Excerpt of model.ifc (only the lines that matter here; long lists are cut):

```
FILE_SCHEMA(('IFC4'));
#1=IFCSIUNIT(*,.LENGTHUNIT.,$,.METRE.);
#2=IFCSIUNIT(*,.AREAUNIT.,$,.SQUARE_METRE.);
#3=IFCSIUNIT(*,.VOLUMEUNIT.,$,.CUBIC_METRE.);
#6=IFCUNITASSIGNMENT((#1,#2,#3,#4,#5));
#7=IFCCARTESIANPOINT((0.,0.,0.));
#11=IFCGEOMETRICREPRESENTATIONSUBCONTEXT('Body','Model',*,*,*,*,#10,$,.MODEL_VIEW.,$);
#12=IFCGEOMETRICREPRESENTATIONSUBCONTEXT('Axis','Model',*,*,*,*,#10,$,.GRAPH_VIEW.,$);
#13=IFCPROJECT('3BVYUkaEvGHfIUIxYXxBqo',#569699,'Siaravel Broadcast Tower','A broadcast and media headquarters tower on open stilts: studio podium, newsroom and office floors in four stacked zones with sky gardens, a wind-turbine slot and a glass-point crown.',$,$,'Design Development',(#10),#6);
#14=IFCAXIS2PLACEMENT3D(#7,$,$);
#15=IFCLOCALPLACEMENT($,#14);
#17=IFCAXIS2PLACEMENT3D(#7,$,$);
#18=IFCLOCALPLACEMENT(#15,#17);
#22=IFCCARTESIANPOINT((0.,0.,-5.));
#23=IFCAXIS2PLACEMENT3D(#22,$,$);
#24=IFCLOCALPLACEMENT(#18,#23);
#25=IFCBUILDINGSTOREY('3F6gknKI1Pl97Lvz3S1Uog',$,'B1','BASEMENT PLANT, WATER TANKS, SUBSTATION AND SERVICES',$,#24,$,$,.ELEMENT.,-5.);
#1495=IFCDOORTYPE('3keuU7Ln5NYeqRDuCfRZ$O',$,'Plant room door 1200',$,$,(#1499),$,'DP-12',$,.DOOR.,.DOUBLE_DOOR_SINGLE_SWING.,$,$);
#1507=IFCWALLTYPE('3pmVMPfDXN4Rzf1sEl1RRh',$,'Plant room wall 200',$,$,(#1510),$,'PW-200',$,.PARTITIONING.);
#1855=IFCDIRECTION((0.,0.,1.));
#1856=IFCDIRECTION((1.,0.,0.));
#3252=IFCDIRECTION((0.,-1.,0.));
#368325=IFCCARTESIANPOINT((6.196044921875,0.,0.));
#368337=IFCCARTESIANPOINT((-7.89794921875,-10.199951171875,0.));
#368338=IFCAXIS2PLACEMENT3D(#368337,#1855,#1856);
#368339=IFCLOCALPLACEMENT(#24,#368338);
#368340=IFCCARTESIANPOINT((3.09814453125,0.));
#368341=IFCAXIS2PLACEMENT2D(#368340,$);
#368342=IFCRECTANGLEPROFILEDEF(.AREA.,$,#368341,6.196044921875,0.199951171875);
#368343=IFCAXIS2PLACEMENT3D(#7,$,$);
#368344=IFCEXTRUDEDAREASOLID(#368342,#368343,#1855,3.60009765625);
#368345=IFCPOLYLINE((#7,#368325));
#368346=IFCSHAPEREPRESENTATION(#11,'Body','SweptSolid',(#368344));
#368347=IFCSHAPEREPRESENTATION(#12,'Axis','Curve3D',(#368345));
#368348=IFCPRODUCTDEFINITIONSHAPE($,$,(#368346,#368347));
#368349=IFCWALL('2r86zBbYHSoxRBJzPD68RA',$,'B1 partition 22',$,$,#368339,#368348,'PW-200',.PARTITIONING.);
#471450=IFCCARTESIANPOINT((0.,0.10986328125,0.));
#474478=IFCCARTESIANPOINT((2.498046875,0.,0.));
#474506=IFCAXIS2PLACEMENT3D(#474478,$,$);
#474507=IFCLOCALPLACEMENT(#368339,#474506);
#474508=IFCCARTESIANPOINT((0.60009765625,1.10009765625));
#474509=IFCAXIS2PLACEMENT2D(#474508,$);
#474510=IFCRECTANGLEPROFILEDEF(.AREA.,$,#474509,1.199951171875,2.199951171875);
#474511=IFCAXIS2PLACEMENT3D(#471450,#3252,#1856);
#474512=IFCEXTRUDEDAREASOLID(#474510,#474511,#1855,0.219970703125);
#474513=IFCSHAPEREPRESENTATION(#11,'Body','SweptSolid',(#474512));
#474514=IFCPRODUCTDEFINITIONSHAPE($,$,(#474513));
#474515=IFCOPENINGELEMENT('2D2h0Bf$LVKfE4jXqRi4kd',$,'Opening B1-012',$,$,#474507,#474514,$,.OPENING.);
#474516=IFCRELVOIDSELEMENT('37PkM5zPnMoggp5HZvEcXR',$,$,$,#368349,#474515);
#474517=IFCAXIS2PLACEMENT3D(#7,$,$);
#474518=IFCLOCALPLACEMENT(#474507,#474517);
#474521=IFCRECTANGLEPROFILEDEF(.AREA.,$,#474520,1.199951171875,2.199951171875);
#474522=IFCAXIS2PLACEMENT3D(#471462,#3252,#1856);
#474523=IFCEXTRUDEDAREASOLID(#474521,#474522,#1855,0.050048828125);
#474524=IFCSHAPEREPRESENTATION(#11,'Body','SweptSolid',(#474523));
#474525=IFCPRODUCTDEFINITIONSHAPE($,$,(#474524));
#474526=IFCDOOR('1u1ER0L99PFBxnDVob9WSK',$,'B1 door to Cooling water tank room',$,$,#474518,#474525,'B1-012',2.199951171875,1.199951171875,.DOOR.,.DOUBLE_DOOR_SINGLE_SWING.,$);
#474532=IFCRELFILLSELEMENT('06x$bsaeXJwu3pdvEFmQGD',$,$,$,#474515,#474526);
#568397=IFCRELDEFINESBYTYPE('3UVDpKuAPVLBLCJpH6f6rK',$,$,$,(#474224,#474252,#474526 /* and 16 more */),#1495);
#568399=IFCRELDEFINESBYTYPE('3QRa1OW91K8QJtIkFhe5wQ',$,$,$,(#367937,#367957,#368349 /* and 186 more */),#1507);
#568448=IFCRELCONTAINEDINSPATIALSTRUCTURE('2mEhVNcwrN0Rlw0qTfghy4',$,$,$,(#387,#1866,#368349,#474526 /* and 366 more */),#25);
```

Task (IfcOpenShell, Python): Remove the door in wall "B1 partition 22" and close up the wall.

```python
import ifcopenshell
import ifcopenshell.api.feature
import ifcopenshell.api.root
import ifcopenshell.geom
import ifcopenshell.util.shape

model = ifcopenshell.open("model.ifc")
settings = ifcopenshell.geom.settings()


def volume(element):
    """Net volume in cubic metres, openings subtracted."""
    shape = ifcopenshell.geom.create_shape(settings, element)
    return ifcopenshell.util.shape.get_volume(shape.geometry)


door = model.by_guid("1u1ER0L99PFBxnDVob9WSK")
opening = door.FillsVoids[0].RelatingOpeningElement
wall = opening.VoidsElements[0].RelatingBuildingElement
before = volume(wall)

ifcopenshell.api.root.remove_product(model, product=door)
ifcopenshell.api.feature.remove_feature(model, feature=opening)

after = volume(wall)

print(f"wall volume {before:.3f} -> {after:.3f} m3")

model.write("model_updated.ifc")
```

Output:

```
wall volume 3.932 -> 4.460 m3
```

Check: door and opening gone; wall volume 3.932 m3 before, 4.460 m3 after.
